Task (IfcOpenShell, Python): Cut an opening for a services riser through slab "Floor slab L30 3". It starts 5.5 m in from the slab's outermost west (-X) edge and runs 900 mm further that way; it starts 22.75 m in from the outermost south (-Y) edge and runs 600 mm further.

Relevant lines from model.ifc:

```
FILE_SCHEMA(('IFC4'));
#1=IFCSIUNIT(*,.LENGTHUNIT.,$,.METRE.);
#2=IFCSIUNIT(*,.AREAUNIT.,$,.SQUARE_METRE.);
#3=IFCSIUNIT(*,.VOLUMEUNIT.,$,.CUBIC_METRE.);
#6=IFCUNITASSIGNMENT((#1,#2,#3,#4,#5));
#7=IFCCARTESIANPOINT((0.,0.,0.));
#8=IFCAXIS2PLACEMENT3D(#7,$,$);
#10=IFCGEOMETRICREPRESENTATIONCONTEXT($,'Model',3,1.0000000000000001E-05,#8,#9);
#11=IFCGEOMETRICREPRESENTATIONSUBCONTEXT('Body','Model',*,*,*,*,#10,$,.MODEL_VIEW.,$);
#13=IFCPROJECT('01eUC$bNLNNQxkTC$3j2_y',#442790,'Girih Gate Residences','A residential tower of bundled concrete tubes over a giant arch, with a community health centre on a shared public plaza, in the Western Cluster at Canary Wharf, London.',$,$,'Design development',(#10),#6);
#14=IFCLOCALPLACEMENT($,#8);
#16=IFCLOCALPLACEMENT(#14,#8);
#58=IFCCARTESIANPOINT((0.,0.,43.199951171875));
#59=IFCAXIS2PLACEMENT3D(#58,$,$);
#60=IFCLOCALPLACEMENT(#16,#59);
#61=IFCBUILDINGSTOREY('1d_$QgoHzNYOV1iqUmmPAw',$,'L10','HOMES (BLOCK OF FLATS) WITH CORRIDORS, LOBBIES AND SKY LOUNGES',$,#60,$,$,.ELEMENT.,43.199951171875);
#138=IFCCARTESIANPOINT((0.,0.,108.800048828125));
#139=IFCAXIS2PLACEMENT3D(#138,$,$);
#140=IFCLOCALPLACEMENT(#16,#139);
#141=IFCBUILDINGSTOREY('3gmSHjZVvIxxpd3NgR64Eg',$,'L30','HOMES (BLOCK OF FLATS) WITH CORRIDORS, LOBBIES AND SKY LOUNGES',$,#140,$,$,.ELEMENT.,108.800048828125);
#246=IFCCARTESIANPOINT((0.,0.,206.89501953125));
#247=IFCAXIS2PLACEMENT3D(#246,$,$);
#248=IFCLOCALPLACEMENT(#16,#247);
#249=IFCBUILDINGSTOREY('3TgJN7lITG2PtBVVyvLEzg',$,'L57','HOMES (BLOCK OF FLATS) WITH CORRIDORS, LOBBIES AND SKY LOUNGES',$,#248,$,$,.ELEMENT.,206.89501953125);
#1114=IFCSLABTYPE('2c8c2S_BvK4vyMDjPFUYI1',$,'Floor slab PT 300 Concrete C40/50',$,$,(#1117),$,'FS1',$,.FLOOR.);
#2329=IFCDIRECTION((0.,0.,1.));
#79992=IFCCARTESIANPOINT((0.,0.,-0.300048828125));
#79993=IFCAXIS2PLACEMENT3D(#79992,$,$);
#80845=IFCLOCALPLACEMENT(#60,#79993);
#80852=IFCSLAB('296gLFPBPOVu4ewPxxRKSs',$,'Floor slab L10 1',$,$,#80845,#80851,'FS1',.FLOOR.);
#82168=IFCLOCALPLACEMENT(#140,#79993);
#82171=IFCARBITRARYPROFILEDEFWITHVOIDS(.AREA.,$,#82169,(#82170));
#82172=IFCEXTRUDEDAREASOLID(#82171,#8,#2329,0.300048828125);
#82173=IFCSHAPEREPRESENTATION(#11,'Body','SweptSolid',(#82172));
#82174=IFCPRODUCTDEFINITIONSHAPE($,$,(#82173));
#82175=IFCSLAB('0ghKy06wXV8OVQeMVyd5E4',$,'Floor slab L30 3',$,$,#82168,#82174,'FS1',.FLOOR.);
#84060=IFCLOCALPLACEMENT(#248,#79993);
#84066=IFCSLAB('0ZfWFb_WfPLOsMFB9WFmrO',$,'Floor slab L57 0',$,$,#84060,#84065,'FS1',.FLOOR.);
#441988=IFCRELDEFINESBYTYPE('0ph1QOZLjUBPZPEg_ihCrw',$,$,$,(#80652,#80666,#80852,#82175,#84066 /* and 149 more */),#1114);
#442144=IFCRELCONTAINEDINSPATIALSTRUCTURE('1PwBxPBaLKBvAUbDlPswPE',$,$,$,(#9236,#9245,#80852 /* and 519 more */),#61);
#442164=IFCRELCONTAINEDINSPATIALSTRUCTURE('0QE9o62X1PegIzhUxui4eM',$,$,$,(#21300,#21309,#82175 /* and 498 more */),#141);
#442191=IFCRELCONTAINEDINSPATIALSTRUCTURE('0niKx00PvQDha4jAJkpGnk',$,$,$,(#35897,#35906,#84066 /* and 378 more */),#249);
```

```python
import numpy as np
import ifcopenshell
import ifcopenshell.api.feature
import ifcopenshell.api.geometry
import ifcopenshell.api.root
import ifcopenshell.geom
import ifcopenshell.util.placement
import ifcopenshell.util.representation
import ifcopenshell.util.shape
import ifcopenshell.util.unit

model = ifcopenshell.open("model.ifc")
unit_scale = ifcopenshell.util.unit.calculate_unit_scale(model)
settings = ifcopenshell.geom.settings()


def volume(element):
    """Net volume in cubic metres, openings subtracted."""
    shape = ifcopenshell.geom.create_shape(settings, element)
    return ifcopenshell.util.shape.get_volume(shape.geometry)


slab = model.by_guid("0ghKy06wXV8OVQeMVyd5E4")
before = volume(slab)

# Extent in the slab's own axes, in metres. The edges named are its -X and -Y sides.
slab_shape = ifcopenshell.geom.create_shape(settings, slab)
vertices = ifcopenshell.util.shape.get_vertices(slab_shape.geometry)
x_min, y_min, bottom = vertices.min(axis=0)
top = vertices[:, 2].max()

opening = ifcopenshell.api.root.create_entity(model, ifc_class="IfcOpeningElement", name="Services riser opening", predefined_type="OPENING")
context = ifcopenshell.util.representation.get_context(model, "Model", "Body", "MODEL_VIEW")
width, depth = 0.9, 0.6
outline = [(0.0, 0.0), (width, 0.0), (width, depth), (0.0, depth), (0.0, 0.0)]
# Overshoot both faces by 50 mm so the cut is clean.
shape = ifcopenshell.api.geometry.add_slab_representation(
    model, context=context, depth=top - bottom + 0.1, polyline=outline
)
ifcopenshell.api.geometry.assign_representation(model, product=opening, representation=shape)

matrix = ifcopenshell.util.placement.get_local_placement(slab.ObjectPlacement)
matrix[:, 3] = matrix @ np.append(np.array([x_min + 5.5, y_min + 22.75, bottom - 0.05]) / unit_scale, 1.0)
ifcopenshell.api.geometry.edit_object_placement(model, product=opening, matrix=matrix, is_si=False)
ifcopenshell.api.feature.add_feature(model, feature=opening, element=slab)

after = volume(slab)

print(f"slab volume {before:.3f} -> {after:.3f} m3")

model.write("model_edited.ifc")
```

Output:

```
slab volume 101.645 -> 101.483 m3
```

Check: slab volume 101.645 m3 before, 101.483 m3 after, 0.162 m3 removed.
